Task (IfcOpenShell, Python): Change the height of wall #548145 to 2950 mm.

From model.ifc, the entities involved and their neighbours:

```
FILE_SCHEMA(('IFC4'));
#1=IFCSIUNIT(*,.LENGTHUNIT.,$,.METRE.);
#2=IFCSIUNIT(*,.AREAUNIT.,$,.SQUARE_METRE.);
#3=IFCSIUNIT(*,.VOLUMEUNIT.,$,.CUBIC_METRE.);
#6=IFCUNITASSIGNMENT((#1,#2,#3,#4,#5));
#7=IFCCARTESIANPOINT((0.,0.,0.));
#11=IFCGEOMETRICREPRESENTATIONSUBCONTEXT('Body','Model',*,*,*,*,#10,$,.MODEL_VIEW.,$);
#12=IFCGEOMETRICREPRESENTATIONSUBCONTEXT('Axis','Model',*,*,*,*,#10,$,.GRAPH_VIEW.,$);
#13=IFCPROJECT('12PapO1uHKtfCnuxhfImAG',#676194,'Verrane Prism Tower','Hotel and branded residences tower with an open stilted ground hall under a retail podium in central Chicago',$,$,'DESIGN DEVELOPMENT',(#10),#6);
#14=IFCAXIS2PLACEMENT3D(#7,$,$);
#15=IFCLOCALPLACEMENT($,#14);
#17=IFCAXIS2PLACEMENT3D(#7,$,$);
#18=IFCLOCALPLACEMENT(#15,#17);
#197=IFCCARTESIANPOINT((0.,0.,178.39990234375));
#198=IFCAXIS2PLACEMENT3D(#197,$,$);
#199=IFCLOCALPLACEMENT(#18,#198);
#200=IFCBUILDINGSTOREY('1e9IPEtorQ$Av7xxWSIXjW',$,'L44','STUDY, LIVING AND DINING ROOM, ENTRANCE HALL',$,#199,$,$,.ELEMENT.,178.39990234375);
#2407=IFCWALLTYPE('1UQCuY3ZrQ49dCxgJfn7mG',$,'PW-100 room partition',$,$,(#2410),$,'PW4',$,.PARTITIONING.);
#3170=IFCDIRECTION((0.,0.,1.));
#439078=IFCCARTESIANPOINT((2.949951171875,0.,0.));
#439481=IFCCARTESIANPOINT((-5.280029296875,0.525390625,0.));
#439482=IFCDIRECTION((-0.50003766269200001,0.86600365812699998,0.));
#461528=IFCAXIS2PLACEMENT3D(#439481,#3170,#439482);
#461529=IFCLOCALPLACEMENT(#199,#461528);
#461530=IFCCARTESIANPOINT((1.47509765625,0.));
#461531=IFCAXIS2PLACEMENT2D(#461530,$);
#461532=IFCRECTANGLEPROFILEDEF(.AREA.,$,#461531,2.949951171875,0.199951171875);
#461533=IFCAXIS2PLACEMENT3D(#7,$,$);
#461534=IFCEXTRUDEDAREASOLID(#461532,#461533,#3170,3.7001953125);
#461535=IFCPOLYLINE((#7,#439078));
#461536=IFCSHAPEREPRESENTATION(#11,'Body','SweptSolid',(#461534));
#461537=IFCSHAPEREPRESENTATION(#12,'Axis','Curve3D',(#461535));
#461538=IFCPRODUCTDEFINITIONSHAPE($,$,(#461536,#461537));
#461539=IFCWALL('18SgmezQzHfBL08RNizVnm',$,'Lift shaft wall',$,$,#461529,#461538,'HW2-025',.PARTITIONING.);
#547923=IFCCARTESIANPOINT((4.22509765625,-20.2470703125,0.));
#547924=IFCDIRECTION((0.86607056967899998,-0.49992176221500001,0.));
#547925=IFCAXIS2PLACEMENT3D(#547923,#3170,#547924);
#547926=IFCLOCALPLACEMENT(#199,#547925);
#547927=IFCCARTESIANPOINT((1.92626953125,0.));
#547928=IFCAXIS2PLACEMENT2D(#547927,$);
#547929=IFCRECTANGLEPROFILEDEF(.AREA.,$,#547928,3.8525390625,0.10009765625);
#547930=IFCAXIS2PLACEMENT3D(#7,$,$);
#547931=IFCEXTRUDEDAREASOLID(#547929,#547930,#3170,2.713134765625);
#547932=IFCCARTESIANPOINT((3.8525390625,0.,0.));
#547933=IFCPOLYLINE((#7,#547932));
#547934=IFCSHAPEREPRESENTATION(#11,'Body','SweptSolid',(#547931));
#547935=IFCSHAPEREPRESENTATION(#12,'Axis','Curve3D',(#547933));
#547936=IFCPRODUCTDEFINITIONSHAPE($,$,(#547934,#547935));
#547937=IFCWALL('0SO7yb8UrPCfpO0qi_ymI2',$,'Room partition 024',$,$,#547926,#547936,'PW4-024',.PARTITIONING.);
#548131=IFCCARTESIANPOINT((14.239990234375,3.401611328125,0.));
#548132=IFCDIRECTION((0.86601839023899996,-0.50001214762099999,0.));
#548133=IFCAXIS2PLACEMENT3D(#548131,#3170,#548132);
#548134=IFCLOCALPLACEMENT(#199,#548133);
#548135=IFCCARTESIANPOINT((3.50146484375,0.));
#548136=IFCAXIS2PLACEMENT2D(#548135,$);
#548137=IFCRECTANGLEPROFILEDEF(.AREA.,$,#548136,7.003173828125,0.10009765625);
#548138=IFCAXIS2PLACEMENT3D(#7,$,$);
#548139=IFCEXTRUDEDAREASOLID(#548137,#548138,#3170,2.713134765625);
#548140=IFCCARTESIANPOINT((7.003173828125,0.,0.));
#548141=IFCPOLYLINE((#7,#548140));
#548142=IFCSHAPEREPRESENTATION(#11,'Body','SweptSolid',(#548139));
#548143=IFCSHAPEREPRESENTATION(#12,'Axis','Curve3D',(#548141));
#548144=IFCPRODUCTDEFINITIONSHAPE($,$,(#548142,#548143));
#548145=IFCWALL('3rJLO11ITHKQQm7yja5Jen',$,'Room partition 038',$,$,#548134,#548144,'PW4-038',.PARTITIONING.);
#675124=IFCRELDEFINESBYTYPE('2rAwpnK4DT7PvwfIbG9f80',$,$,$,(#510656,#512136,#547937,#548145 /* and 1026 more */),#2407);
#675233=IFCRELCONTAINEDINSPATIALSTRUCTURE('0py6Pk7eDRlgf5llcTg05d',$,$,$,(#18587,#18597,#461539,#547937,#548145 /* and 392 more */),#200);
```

```python
import ifcopenshell
import ifcopenshell.geom
import ifcopenshell.util.representation
import ifcopenshell.util.shape
import ifcopenshell.util.unit

model = ifcopenshell.open("model.ifc")
unit_scale = ifcopenshell.util.unit.calculate_unit_scale(model)
settings = ifcopenshell.geom.settings()


def volume(element):
    """Net volume in cubic metres, openings subtracted."""
    shape = ifcopenshell.geom.create_shape(settings, element)
    return ifcopenshell.util.shape.get_volume(shape.geometry)


wall = model.by_id(548145)
before = volume(wall)

body = ifcopenshell.util.representation.get_representation(wall, "Model", "Body")
solid = body.Items[0]
old_height = solid.Depth
solid.Depth = 2.95 / unit_scale
after = volume(wall)

print(f"height {old_height:g} -> {solid.Depth:g}, volume {before:.3f} -> {after:.3f} m3")

model.write("model_rev.ifc")
```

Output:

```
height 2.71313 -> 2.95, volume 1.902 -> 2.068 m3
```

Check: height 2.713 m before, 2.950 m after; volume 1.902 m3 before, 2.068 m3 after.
